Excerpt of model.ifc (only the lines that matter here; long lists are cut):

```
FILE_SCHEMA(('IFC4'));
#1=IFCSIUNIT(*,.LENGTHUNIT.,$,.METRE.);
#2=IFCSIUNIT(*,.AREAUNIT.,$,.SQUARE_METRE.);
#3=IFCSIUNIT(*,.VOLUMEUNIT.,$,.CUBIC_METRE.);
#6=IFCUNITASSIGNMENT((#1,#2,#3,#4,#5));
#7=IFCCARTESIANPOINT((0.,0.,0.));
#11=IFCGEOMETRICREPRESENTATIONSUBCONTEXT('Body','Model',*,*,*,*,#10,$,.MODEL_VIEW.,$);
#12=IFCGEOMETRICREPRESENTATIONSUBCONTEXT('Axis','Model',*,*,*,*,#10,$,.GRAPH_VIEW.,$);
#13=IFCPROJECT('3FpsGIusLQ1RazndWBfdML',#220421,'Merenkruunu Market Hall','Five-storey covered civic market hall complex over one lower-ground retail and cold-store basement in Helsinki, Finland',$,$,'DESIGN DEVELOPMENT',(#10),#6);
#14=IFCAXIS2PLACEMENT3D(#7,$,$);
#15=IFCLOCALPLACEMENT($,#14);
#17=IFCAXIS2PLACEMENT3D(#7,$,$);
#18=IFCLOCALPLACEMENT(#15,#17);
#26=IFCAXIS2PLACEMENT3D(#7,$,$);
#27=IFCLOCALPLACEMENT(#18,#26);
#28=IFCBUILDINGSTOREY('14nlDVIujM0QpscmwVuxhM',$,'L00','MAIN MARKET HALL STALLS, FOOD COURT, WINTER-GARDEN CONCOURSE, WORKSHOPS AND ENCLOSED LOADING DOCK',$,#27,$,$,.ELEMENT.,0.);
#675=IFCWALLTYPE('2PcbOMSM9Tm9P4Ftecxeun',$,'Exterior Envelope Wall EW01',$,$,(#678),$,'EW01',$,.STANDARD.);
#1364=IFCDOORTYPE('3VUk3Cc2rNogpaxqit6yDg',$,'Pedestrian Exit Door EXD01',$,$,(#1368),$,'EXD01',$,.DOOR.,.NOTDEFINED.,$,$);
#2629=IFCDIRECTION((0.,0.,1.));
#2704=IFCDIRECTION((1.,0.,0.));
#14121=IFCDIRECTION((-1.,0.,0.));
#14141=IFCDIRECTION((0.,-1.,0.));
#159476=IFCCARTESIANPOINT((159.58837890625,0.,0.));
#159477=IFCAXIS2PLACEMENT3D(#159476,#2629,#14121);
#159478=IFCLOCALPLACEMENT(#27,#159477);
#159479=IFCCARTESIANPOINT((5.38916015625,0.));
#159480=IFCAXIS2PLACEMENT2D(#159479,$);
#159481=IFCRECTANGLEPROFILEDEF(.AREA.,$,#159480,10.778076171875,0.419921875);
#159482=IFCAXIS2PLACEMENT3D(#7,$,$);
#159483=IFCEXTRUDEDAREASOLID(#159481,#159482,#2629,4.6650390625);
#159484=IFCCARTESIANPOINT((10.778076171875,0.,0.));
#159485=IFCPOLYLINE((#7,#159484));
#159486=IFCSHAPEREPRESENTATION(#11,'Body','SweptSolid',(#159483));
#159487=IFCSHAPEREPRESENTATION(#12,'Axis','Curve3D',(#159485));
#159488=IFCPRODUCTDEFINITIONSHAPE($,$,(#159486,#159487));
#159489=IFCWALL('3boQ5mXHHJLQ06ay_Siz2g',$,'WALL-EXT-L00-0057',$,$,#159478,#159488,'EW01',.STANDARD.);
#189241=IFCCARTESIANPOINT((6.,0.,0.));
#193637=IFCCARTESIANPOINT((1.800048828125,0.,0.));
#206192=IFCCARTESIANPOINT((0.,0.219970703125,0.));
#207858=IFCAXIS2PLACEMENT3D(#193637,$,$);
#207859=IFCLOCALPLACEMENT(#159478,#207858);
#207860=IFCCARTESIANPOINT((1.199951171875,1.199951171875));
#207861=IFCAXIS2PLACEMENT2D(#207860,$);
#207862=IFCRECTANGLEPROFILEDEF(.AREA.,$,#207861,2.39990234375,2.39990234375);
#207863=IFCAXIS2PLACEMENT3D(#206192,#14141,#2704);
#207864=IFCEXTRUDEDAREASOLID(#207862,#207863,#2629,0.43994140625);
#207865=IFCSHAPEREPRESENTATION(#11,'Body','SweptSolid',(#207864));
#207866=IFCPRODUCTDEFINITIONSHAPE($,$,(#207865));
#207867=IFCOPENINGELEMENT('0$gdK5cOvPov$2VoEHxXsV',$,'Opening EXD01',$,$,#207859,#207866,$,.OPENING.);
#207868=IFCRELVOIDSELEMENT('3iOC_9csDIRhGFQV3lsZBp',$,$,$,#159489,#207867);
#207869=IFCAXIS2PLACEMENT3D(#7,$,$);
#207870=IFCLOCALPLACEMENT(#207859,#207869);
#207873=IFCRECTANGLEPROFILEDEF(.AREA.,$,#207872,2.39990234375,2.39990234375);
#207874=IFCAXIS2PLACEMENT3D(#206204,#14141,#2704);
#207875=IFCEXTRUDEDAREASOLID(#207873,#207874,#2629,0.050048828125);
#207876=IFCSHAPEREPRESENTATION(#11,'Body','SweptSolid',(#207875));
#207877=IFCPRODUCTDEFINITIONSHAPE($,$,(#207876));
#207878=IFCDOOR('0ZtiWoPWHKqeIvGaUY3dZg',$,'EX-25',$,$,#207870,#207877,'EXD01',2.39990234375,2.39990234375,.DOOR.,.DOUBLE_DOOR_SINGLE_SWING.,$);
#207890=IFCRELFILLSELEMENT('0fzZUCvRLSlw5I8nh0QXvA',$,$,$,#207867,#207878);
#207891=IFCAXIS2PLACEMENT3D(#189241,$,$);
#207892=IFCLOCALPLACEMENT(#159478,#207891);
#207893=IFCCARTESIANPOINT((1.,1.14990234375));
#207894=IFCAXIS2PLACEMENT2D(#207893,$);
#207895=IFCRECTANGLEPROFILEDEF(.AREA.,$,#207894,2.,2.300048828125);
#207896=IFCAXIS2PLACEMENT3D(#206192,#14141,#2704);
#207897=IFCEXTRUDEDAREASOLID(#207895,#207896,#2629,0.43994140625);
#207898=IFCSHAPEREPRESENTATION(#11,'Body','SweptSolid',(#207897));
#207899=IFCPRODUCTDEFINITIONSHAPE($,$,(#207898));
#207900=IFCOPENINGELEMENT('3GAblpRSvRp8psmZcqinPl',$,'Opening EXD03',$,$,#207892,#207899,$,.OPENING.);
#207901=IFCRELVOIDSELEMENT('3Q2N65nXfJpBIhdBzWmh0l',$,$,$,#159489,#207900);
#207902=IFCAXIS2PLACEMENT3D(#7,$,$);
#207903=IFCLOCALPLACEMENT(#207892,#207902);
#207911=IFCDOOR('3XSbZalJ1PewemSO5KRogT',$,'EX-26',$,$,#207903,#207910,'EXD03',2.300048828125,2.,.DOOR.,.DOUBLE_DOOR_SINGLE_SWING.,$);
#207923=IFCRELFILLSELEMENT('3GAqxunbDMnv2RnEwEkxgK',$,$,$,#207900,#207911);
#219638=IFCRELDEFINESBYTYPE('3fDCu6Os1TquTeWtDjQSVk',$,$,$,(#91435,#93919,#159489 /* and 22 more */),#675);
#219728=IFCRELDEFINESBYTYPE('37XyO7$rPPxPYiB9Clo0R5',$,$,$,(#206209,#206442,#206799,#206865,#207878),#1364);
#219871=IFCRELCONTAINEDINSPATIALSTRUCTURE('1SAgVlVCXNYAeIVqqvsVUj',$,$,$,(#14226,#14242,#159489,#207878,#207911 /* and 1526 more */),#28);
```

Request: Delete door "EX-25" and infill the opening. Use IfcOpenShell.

```python
import ifcopenshell
import ifcopenshell.api.feature
import ifcopenshell.api.root
import ifcopenshell.geom
import ifcopenshell.util.shape

model = ifcopenshell.open("model.ifc")
settings = ifcopenshell.geom.settings()


def volume(element):
    """Net volume in cubic metres, openings subtracted."""
    shape = ifcopenshell.geom.create_shape(settings, element)
    return ifcopenshell.util.shape.get_volume(shape.geometry)


door = model.by_id(207878)
opening = door.FillsVoids[0].RelatingOpeningElement
wall = opening.VoidsElements[0].RelatingBuildingElement
before = volume(wall)

ifcopenshell.api.root.remove_product(model, product=door)
ifcopenshell.api.feature.remove_feature(model, feature=opening)

after = volume(wall)

print(f"wall volume {before:.3f} -> {after:.3f} m3")

model.write("model_updated.ifc")
```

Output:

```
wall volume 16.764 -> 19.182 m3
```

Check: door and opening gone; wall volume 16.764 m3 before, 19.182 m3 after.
